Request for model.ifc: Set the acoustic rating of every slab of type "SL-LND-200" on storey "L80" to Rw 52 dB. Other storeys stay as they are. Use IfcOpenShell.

First a look at what the model holds.

```python
import ifcopenshell
import ifcopenshell.util.element

model = ifcopenshell.open("model.ifc")
print(model.schema)
storey = next(s for s in model.by_type("IfcBuildingStorey") if s.Name == "L80")
slabs = [e for e in ifcopenshell.util.element.get_decomposition(storey) if e.is_a("IfcSlab")]
seen = {}
for e in slabs:
    element_type = ifcopenshell.util.element.get_type(e)
    key = (element_type.Name if element_type != e and element_type else None, ifcopenshell.util.element.get_pset(e, "Pset_SlabCommon", "AcousticRating"))
    seen[key] = seen.get(key, 0) + 1
for (name, value), count in sorted(seen.items(), key=str):
    print(count, "x", name, "|", value)
```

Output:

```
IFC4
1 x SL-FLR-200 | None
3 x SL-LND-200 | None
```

```python
import ifcopenshell
import ifcopenshell.api.pset
import ifcopenshell.util.element

model = ifcopenshell.open("model.ifc")

storey = next(s for s in model.by_type("IfcBuildingStorey") if s.Name == "L80")
slabs = [e for e in ifcopenshell.util.element.get_decomposition(storey) if e.is_a("IfcSlab")]

count = 0
for e in slabs:
    element_type = ifcopenshell.util.element.get_type(e)
    if element_type in (None, e) or element_type.Name != "SL-LND-200":
        continue
    # add_pset returns the element's existing set when there is one.
    pset = ifcopenshell.api.pset.add_pset(model, product=e, name="Pset_SlabCommon")
    ifcopenshell.api.pset.edit_pset(model, pset=pset, properties={"AcousticRating": "Rw 52 dB"})
    count += 1

print(count, "slabs updated")

model.write("model_v2.ifc")
```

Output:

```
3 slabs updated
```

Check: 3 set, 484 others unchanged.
